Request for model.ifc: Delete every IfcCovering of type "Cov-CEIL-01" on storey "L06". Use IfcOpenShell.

First a look at what the model holds.

```python
import ifcopenshell
import ifcopenshell.util.element

model = ifcopenshell.open("model.ifc")
print(model.schema)
storey = next(s for s in model.by_type("IfcBuildingStorey") if s.Name == "L06")
coverings = [e for e in ifcopenshell.util.element.get_decomposition(storey) if e.is_a("IfcCovering")]
seen = {}
for e in coverings:
    element_type = ifcopenshell.util.element.get_type(e)
    name = element_type.Name if element_type not in (None, e) else None
    seen[name] = seen.get(name, 0) + 1
for name, count in sorted(seen.items(), key=str):
    print(count, "x", name)
```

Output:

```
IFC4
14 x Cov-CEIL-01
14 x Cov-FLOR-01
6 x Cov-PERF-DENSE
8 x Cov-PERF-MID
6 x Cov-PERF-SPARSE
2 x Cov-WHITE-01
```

```python
import ifcopenshell
import ifcopenshell.api.root
import ifcopenshell.util.element

model = ifcopenshell.open("model.ifc")

storey = next(s for s in model.by_type("IfcBuildingStorey") if s.Name == "L06")
coverings = [e for e in ifcopenshell.util.element.get_decomposition(storey) if e.is_a("IfcCovering")]
targets = [e for e in coverings if (t := ifcopenshell.util.element.get_type(e)) not in (None, e) and t.Name == "Cov-CEIL-01"]

for e in targets:
    ifcopenshell.api.root.remove_product(model, product=e)
print(len(targets), "removed")

model.write("model_rev.ifc")
```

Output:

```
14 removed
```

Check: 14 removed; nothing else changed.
